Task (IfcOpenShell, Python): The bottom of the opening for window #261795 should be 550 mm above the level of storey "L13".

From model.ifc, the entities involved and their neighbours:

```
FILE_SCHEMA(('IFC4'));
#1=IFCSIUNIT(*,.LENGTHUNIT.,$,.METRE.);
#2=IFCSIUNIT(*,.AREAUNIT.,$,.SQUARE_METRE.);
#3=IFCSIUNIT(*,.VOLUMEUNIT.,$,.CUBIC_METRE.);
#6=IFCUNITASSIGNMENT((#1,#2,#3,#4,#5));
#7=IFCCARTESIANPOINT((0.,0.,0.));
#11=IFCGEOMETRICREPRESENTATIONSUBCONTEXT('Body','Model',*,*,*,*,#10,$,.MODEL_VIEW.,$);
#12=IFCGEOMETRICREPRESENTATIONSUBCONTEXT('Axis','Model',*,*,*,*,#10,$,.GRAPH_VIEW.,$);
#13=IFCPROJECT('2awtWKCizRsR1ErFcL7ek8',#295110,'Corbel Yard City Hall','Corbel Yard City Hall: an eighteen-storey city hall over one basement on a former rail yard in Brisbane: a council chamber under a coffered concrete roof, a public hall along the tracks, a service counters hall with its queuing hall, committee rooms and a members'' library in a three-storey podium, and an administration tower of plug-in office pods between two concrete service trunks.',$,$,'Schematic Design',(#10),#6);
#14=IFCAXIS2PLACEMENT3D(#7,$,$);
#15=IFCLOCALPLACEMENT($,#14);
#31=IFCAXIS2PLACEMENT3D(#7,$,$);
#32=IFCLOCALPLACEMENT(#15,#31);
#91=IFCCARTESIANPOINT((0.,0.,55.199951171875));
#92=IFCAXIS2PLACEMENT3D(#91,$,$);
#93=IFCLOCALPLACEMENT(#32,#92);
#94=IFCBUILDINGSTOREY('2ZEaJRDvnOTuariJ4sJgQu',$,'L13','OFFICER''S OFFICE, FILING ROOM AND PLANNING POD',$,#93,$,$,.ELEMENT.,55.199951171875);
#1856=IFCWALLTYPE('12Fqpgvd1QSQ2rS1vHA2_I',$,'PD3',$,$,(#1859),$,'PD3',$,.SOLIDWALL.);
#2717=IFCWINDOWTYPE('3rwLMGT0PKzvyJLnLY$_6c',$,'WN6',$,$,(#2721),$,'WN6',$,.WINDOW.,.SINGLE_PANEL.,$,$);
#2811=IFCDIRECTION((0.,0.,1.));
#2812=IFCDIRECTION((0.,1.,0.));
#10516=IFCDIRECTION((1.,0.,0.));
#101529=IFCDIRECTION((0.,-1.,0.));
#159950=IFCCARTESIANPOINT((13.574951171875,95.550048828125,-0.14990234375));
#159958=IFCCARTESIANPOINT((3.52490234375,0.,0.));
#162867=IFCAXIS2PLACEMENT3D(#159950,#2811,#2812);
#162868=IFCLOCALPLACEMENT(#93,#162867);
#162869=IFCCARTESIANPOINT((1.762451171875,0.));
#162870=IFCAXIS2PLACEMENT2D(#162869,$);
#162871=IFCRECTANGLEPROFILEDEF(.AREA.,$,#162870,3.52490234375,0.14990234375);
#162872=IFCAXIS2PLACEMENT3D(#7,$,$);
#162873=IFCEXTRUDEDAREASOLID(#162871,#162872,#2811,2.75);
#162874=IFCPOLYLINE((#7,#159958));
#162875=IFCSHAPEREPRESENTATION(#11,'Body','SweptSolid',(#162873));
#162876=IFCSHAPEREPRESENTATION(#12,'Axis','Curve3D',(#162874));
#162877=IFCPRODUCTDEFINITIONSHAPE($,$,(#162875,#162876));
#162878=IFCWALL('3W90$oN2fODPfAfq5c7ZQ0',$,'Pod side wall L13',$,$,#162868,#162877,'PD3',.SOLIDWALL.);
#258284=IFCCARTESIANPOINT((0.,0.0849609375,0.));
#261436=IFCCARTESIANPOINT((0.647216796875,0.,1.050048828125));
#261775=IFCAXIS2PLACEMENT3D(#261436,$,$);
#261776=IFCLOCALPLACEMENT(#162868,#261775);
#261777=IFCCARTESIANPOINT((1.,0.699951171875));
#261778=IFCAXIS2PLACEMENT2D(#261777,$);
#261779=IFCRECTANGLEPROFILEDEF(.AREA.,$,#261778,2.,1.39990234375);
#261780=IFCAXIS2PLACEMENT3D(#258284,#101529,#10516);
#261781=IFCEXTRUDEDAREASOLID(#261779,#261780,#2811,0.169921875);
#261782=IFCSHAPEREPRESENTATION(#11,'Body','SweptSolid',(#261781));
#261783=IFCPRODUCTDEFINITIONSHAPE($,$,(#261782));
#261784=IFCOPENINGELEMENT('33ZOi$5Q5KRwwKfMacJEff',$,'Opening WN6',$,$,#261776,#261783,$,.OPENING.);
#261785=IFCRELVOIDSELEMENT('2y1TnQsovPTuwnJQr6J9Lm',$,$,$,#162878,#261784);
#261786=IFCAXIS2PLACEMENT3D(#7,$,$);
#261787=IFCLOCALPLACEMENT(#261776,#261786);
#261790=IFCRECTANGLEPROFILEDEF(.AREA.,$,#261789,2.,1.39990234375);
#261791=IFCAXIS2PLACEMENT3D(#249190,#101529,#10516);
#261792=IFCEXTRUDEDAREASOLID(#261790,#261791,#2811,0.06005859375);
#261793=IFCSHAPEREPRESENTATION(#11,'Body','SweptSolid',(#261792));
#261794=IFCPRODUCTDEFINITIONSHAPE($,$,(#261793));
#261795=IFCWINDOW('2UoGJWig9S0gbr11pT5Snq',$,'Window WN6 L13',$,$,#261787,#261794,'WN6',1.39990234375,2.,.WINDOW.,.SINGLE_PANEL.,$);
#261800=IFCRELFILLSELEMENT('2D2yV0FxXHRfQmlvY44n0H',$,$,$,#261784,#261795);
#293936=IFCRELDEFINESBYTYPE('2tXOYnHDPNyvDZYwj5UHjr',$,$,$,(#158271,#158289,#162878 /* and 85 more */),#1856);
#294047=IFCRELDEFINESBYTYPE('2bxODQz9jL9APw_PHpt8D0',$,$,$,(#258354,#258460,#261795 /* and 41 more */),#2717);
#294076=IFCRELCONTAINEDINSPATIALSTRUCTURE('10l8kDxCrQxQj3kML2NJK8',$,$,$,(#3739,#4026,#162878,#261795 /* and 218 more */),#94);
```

```python
import numpy as np
import ifcopenshell
import ifcopenshell.api.geometry
import ifcopenshell.geom
import ifcopenshell.util.element
import ifcopenshell.util.placement
import ifcopenshell.util.shape
import ifcopenshell.util.unit

model = ifcopenshell.open("model.ifc")
unit_scale = ifcopenshell.util.unit.calculate_unit_scale(model)

window = model.by_id(261795)
opening = window.FillsVoids[0].RelatingOpeningElement
storey = ifcopenshell.util.element.get_container(window, ifc_class="IfcBuildingStorey")
level = ifcopenshell.util.placement.get_local_placement(storey.ObjectPlacement)[2, 3]

# The opening's origin need not be at the sill, so measure its lowest point.
shape = ifcopenshell.geom.create_shape(ifcopenshell.geom.settings(), opening)
bottom = ifcopenshell.util.shape.get_shape_bottom_elevation(shape, shape.geometry) / unit_scale
dz = level + 0.55 / unit_scale - bottom

shift = np.array([0.0, 0.0, dz])
# The window is placed relative to its opening, so it follows when the opening moves.
matrix = ifcopenshell.util.placement.get_local_placement(opening.ObjectPlacement)
matrix[:3, 3] += shift
ifcopenshell.api.geometry.edit_object_placement(
    model, product=opening, matrix=matrix, is_si=False, should_transform_children=True
)

print(f"moved by {dz * unit_scale:+.3f} m")

model.write("model_rev.ifc")
```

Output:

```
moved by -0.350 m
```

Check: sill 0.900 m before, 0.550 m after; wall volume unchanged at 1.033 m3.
